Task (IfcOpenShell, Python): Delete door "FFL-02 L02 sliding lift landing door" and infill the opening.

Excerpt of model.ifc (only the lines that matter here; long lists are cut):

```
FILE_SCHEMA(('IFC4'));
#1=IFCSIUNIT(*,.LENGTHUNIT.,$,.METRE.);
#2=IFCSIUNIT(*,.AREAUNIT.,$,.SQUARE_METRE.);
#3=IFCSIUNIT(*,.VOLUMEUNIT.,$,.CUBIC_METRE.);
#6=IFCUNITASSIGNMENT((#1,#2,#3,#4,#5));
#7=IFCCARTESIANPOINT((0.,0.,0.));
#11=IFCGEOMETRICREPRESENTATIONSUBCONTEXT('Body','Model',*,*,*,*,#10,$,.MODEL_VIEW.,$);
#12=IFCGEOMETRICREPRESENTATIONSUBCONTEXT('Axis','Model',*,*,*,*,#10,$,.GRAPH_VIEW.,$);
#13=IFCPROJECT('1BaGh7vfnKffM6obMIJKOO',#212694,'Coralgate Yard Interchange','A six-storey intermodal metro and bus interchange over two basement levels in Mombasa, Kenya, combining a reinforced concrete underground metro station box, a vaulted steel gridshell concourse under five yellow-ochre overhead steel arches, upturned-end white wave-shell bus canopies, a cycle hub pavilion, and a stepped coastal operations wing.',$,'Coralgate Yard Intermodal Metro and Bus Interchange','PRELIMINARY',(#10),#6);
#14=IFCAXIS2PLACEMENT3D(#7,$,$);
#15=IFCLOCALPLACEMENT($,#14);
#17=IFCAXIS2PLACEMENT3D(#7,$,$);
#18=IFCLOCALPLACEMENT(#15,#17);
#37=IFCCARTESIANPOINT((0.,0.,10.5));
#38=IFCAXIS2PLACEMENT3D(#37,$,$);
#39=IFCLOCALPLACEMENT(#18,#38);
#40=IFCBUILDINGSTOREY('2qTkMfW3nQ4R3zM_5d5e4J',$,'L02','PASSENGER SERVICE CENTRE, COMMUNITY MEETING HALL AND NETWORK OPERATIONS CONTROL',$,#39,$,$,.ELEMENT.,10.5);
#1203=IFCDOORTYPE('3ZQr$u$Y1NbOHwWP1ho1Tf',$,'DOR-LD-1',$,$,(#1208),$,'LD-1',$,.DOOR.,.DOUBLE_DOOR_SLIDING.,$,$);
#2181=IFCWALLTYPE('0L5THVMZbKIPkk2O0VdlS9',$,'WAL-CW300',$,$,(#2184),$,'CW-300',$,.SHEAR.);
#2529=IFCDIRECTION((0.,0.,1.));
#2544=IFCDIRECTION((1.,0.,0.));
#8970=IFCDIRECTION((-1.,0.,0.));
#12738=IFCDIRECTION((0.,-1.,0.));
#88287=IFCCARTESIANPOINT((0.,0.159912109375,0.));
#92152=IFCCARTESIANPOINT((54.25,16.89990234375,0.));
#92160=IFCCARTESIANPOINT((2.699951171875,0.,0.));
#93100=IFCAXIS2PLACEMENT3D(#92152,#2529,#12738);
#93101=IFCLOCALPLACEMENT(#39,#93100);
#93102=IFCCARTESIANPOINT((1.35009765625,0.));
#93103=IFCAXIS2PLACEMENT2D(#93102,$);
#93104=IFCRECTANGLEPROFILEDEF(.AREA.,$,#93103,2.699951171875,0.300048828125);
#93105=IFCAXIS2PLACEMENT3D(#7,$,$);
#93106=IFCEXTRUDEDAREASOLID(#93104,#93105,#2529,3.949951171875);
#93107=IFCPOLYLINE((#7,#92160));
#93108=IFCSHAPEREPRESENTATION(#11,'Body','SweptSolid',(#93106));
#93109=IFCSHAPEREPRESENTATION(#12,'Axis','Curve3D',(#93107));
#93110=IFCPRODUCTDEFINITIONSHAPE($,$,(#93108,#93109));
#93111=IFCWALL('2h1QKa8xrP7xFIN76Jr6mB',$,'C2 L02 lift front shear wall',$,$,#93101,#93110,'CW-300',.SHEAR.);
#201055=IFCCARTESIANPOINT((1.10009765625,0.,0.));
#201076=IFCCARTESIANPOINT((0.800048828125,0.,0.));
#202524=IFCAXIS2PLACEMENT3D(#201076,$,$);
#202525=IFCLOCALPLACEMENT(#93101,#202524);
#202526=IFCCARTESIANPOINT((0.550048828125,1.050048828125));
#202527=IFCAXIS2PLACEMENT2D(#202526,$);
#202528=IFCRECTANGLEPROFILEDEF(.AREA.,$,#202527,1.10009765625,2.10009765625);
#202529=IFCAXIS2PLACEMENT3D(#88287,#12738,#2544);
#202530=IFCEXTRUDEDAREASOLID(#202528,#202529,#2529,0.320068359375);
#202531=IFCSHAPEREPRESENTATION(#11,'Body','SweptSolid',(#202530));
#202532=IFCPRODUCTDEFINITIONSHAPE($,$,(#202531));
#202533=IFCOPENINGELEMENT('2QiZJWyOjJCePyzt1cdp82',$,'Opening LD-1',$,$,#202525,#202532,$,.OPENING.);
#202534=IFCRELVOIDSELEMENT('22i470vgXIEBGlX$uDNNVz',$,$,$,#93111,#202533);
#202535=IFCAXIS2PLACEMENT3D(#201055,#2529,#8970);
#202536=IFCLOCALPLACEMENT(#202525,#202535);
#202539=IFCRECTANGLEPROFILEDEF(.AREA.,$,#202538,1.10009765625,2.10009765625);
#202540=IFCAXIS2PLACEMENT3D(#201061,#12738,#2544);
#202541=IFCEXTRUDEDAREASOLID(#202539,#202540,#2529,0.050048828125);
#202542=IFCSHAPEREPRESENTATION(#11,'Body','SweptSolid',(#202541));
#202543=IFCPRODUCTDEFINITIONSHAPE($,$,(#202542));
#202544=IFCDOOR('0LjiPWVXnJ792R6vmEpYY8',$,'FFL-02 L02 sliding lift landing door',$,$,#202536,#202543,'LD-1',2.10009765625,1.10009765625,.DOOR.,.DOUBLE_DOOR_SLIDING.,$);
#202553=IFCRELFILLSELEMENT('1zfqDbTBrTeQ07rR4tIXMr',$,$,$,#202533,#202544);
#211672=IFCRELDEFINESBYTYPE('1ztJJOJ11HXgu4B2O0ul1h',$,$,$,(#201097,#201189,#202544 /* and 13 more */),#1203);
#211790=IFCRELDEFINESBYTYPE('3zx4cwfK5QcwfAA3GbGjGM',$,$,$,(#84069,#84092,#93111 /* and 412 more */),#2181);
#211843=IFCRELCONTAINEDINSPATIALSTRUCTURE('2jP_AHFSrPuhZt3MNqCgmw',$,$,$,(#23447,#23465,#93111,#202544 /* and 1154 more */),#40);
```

```python
import ifcopenshell
import ifcopenshell.api.feature
import ifcopenshell.api.root
import ifcopenshell.geom
import ifcopenshell.util.shape

model = ifcopenshell.open("model.ifc")
settings = ifcopenshell.geom.settings()


def volume(element):
    """Net volume in cubic metres, openings subtracted."""
    shape = ifcopenshell.geom.create_shape(settings, element)
    return ifcopenshell.util.shape.get_volume(shape.geometry)


door = model.by_guid("0LjiPWVXnJ792R6vmEpYY8")
opening = door.FillsVoids[0].RelatingOpeningElement
wall = opening.VoidsElements[0].RelatingBuildingElement
before = volume(wall)

ifcopenshell.api.root.remove_product(model, product=door)
ifcopenshell.api.feature.remove_feature(model, feature=opening)

after = volume(wall)

print(f"wall volume {before:.3f} -> {after:.3f} m3")

model.write("model_rev.ifc")
```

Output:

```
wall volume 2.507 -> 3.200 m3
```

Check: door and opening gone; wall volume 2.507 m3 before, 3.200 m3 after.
